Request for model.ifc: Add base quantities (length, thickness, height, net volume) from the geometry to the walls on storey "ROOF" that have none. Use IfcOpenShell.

First a look at what the model holds.

```python
import ifcopenshell
import ifcopenshell.util.element
import ifcopenshell.util.unit

model = ifcopenshell.open("model.ifc")
print(model.schema)
for unit_type in ("LENGTHUNIT", "AREAUNIT", "VOLUMEUNIT"):
    print(unit_type, ifcopenshell.util.unit.calculate_unit_scale(model, unit_type))
storey = next(s for s in model.by_type("IfcBuildingStorey") if s.Name == "ROOF")
walls = [e for e in ifcopenshell.util.element.get_decomposition(storey) if e.is_a("IfcWall")]
for e in sorted(walls, key=lambda e: e.id()):
    print(e.id(), e.is_a(), e.Name, list(ifcopenshell.util.element.get_psets(e, qtos_only=True)), sep=" | ")
```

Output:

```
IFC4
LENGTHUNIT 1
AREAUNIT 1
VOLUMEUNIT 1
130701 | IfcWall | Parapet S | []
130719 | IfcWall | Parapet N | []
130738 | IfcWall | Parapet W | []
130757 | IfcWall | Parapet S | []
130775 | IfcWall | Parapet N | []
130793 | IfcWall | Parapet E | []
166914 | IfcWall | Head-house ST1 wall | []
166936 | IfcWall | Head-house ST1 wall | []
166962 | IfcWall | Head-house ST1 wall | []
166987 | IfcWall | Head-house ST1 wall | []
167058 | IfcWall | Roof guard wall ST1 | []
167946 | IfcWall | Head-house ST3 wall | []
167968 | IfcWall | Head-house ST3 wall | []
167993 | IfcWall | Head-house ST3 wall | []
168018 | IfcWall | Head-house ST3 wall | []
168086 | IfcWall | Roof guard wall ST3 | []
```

```python
import ifcopenshell
import ifcopenshell.api.pset
import ifcopenshell.geom
import ifcopenshell.util.element
import ifcopenshell.util.shape
import ifcopenshell.util.unit

model = ifcopenshell.open("model.ifc")
unit_scale = ifcopenshell.util.unit.calculate_unit_scale(model)
volume_scale = ifcopenshell.util.unit.calculate_unit_scale(model, "VOLUMEUNIT")
settings = ifcopenshell.geom.settings()

storey = next(s for s in model.by_type("IfcBuildingStorey") if s.Name == "ROOF")
walls = [e for e in ifcopenshell.util.element.get_decomposition(storey) if e.is_a("IfcWall")]

for e in sorted(walls, key=lambda e: e.id()):
    if ifcopenshell.util.element.get_psets(e, qtos_only=True, should_inherit=False):
        continue
    # Geometry comes back in metres, in the element's own axes.
    shape = ifcopenshell.geom.create_shape(settings, e)
    values = {
        "Length": ifcopenshell.util.shape.get_x(shape.geometry) / unit_scale,
        "Width": ifcopenshell.util.shape.get_y(shape.geometry) / unit_scale,
        "Height": ifcopenshell.util.shape.get_z(shape.geometry) / unit_scale,
        "NetVolume": ifcopenshell.util.shape.get_volume(shape.geometry) / volume_scale,
    }
    qto = ifcopenshell.api.pset.add_qto(model, product=e, name="Qto_WallBaseQuantities")
    ifcopenshell.api.pset.edit_qto(model, qto=qto, properties=values)
    print(e.id(), {k: round(v, 3) for k, v in values.items()})

model.write("model_v2.ifc")
```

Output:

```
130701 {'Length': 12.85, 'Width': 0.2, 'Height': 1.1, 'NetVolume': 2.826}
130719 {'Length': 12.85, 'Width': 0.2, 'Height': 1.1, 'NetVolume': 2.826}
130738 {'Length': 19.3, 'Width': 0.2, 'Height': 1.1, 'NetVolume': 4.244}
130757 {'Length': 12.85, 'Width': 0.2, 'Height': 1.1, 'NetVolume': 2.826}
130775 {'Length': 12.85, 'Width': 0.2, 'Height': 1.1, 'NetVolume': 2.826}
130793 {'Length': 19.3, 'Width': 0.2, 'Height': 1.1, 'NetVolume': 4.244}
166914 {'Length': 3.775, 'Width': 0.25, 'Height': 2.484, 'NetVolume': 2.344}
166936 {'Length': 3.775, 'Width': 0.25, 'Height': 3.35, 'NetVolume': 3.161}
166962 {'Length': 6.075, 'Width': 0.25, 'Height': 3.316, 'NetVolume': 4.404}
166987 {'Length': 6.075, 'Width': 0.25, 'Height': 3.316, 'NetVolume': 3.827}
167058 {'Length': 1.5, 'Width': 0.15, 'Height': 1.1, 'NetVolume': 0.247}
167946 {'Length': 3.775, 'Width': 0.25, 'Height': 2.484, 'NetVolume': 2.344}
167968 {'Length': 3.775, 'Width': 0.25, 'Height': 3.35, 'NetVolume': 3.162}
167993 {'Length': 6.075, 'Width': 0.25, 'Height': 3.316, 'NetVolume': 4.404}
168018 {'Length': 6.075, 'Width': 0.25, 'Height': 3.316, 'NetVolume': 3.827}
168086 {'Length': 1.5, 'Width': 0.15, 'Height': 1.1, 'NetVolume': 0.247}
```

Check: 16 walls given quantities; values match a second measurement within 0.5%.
